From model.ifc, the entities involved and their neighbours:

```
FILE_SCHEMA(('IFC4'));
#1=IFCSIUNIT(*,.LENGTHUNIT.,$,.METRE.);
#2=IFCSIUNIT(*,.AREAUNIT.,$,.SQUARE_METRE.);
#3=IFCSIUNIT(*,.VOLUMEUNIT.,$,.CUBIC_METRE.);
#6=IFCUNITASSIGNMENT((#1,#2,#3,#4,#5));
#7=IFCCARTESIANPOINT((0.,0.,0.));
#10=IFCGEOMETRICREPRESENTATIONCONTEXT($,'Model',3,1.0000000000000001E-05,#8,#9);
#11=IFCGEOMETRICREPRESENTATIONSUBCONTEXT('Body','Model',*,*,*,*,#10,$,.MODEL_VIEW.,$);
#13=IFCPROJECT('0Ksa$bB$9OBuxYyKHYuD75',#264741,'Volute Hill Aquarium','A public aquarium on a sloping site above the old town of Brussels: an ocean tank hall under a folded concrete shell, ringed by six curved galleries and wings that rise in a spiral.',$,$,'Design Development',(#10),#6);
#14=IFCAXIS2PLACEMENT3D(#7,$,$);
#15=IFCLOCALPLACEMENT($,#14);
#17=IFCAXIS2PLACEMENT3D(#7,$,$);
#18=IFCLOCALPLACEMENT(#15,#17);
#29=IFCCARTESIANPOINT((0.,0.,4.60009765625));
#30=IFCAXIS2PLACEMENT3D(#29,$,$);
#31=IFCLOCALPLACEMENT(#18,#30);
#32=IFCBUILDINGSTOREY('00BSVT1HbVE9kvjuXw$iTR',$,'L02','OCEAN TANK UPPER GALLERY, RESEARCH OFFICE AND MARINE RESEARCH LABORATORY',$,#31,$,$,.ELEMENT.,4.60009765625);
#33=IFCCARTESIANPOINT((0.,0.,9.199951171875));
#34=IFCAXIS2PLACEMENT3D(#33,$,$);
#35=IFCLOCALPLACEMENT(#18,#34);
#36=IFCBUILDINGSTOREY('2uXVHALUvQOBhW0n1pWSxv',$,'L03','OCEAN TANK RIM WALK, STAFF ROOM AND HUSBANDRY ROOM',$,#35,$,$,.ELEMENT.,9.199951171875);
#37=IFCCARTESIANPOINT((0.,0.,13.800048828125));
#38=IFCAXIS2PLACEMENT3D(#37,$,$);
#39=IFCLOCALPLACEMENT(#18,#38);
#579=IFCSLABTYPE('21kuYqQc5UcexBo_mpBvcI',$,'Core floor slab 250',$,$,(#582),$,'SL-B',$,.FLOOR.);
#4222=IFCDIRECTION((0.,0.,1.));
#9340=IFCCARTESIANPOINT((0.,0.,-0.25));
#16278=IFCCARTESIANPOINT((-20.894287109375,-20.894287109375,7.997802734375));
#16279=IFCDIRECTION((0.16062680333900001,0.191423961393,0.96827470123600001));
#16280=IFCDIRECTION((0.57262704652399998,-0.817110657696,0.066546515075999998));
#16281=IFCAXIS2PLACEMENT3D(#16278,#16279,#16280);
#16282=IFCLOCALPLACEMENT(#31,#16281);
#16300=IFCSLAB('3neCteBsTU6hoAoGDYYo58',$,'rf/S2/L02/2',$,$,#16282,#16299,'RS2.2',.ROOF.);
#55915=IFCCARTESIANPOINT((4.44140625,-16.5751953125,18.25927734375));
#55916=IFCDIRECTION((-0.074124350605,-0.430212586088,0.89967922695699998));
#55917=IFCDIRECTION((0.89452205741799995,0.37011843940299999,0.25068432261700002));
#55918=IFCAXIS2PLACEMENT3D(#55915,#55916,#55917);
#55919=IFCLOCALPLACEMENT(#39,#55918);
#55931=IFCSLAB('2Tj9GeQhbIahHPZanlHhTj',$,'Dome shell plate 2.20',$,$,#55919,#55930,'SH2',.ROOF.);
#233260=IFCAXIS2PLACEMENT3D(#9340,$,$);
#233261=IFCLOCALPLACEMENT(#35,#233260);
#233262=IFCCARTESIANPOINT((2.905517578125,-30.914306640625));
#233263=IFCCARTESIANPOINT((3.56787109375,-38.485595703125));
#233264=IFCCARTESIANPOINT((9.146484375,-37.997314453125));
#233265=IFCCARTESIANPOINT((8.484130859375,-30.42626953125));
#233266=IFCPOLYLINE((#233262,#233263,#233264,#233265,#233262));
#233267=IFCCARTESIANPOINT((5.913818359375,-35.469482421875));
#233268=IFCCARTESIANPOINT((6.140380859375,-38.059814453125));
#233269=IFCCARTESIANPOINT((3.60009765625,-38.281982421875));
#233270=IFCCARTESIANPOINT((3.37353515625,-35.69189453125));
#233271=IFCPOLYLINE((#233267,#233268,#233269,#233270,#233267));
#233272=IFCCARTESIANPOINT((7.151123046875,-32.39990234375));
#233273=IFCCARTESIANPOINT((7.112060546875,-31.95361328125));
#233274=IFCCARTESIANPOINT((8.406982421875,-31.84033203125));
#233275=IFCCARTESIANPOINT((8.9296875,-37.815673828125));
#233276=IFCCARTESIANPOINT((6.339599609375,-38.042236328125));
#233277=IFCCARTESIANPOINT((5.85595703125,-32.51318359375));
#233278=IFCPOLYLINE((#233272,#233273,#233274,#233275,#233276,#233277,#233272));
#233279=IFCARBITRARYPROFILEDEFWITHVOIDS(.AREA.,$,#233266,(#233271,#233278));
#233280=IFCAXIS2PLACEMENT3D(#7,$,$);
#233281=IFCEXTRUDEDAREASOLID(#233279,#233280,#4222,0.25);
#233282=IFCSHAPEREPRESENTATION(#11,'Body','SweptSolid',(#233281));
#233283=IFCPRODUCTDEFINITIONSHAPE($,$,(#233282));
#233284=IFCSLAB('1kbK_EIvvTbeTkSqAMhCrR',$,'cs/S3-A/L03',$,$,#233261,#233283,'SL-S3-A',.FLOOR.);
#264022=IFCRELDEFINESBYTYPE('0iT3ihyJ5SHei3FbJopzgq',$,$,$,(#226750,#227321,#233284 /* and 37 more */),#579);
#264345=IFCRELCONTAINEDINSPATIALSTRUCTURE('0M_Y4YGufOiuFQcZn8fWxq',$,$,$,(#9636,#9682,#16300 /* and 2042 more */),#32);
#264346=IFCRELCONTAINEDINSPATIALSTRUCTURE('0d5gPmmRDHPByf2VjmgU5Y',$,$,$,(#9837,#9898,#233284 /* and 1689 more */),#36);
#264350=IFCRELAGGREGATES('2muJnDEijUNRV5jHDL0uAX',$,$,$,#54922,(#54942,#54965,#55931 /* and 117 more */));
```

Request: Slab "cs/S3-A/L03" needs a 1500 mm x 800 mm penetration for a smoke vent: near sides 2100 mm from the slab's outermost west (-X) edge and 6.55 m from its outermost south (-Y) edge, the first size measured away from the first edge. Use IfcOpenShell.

```python
import numpy as np
import ifcopenshell
import ifcopenshell.api.feature
import ifcopenshell.api.geometry
import ifcopenshell.api.root
import ifcopenshell.geom
import ifcopenshell.util.placement
import ifcopenshell.util.representation
import ifcopenshell.util.shape
import ifcopenshell.util.unit

model = ifcopenshell.open("model.ifc")
unit_scale = ifcopenshell.util.unit.calculate_unit_scale(model)
settings = ifcopenshell.geom.settings()


def volume(element):
    """Net volume in cubic metres, openings subtracted."""
    shape = ifcopenshell.geom.create_shape(settings, element)
    return ifcopenshell.util.shape.get_volume(shape.geometry)


slab = model.by_guid("1kbK_EIvvTbeTkSqAMhCrR")
before = volume(slab)

# Extent in the slab's own axes, in metres. The edges named are its -X and -Y sides.
slab_shape = ifcopenshell.geom.create_shape(settings, slab)
vertices = ifcopenshell.util.shape.get_vertices(slab_shape.geometry)
x_min, y_min, bottom = vertices.min(axis=0)
top = vertices[:, 2].max()

opening = ifcopenshell.api.root.create_entity(model, ifc_class="IfcOpeningElement", name="Smoke vent opening", predefined_type="OPENING")
context = ifcopenshell.util.representation.get_context(model, "Model", "Body", "MODEL_VIEW")
width, depth = 1.5, 0.8
outline = [(0.0, 0.0), (width, 0.0), (width, depth), (0.0, depth), (0.0, 0.0)]
# Overshoot both faces by 50 mm so the cut is clean.
shape = ifcopenshell.api.geometry.add_slab_representation(
    model, context=context, depth=top - bottom + 0.1, polyline=outline
)
ifcopenshell.api.geometry.assign_representation(model, product=opening, representation=shape)

matrix = ifcopenshell.util.placement.get_local_placement(slab.ObjectPlacement)
matrix[:, 3] = matrix @ np.append(np.array([x_min + 2.1, y_min + 6.55, bottom - 0.05]) / unit_scale, 1.0)
ifcopenshell.api.geometry.edit_object_placement(model, product=opening, matrix=matrix, is_si=False)
ifcopenshell.api.feature.add_feature(model, feature=opening, element=slab)

after = volume(slab)

print(f"slab volume {before:.3f} -> {after:.3f} m3")

model.write("model_updated.ifc")
```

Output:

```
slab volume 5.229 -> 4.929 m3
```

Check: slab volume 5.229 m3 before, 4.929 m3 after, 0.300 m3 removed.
